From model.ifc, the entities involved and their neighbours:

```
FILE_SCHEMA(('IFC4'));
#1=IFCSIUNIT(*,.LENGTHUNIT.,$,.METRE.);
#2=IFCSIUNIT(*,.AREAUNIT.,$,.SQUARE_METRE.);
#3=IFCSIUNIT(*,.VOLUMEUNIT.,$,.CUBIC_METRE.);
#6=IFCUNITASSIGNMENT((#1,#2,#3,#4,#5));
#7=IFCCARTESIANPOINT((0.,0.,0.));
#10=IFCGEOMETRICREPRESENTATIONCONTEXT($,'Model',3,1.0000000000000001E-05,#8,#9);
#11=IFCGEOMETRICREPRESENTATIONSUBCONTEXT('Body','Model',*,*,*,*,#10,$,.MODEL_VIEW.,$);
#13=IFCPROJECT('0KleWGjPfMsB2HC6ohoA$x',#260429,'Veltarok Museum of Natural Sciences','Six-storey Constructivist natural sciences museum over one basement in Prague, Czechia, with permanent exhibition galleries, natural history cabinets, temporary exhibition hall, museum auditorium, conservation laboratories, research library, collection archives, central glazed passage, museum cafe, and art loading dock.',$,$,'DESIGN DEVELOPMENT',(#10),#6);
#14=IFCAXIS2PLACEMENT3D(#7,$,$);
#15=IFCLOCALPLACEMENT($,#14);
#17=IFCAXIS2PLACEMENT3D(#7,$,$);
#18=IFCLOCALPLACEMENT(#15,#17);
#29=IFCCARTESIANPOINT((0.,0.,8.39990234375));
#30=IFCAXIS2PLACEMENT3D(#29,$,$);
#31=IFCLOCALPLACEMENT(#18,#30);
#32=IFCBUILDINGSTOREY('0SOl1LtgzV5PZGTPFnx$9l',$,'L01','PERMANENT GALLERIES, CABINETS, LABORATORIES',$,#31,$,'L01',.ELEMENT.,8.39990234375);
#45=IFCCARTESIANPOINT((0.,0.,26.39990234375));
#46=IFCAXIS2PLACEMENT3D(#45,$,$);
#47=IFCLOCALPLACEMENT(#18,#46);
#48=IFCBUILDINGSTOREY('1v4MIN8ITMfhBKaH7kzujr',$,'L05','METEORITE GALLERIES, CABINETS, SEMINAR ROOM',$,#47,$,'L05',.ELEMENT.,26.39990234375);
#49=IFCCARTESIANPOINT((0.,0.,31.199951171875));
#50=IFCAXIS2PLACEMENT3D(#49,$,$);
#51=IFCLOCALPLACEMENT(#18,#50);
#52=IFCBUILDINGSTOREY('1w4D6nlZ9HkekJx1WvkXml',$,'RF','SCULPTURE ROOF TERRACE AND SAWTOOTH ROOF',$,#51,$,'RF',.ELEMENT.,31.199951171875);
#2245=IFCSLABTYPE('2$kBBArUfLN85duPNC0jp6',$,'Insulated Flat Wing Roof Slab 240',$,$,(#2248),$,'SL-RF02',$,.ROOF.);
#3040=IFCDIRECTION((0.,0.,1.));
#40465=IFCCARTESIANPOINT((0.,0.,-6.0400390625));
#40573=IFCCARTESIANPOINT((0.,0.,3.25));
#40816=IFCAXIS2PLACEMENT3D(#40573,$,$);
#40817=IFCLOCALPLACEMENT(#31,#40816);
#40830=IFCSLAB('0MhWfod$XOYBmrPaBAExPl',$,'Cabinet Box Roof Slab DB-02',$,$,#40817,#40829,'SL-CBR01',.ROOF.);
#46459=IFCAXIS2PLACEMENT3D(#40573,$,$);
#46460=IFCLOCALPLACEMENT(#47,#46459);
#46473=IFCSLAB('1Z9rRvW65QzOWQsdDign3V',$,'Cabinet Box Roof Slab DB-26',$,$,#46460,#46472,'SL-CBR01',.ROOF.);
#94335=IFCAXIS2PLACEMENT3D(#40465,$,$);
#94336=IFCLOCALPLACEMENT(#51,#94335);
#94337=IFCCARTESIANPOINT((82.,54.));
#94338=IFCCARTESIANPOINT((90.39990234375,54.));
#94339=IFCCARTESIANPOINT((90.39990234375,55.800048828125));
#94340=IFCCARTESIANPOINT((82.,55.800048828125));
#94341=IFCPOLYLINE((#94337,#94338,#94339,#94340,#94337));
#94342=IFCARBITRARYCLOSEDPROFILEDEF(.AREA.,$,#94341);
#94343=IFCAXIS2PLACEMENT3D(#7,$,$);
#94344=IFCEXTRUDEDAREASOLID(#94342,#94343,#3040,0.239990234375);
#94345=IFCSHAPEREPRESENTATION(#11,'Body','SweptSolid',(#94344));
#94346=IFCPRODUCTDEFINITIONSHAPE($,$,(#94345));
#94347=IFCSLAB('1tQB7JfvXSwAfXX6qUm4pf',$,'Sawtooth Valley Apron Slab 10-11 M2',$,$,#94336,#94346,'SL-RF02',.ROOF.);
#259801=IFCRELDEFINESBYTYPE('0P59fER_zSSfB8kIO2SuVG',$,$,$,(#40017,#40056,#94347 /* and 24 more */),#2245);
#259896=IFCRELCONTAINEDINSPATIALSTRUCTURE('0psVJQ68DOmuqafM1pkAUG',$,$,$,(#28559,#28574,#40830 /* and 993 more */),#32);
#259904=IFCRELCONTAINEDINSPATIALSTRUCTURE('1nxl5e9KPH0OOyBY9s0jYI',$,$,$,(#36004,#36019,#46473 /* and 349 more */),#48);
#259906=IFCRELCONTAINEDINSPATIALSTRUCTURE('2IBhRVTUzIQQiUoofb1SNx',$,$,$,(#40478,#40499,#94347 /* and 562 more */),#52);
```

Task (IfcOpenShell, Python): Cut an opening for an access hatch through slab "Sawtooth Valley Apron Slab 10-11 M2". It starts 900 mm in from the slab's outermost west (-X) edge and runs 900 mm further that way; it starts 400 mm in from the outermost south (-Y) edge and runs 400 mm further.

```python
import numpy as np
import ifcopenshell
import ifcopenshell.api.feature
import ifcopenshell.api.geometry
import ifcopenshell.api.root
import ifcopenshell.geom
import ifcopenshell.util.placement
import ifcopenshell.util.representation
import ifcopenshell.util.shape
import ifcopenshell.util.unit

model = ifcopenshell.open("model.ifc")
unit_scale = ifcopenshell.util.unit.calculate_unit_scale(model)
settings = ifcopenshell.geom.settings()


def volume(element):
    """Net volume in cubic metres, openings subtracted."""
    shape = ifcopenshell.geom.create_shape(settings, element)
    return ifcopenshell.util.shape.get_volume(shape.geometry)


slab = model.by_guid("1tQB7JfvXSwAfXX6qUm4pf")
before = volume(slab)

# Extent in the slab's own axes, in metres. The edges named are its -X and -Y sides.
slab_shape = ifcopenshell.geom.create_shape(settings, slab)
vertices = ifcopenshell.util.shape.get_vertices(slab_shape.geometry)
x_min, y_min, bottom = vertices.min(axis=0)
top = vertices[:, 2].max()

opening = ifcopenshell.api.root.create_entity(model, ifc_class="IfcOpeningElement", name="Access hatch opening", predefined_type="OPENING")
context = ifcopenshell.util.representation.get_context(model, "Model", "Body", "MODEL_VIEW")
width, depth = 0.9, 0.4
outline = [(0.0, 0.0), (width, 0.0), (width, depth), (0.0, depth), (0.0, 0.0)]
# Overshoot both faces by 50 mm so the cut is clean.
shape = ifcopenshell.api.geometry.add_slab_representation(
    model, context=context, depth=top - bottom + 0.1, polyline=outline
)
ifcopenshell.api.geometry.assign_representation(model, product=opening, representation=shape)

matrix = ifcopenshell.util.placement.get_local_placement(slab.ObjectPlacement)
matrix[:, 3] = matrix @ np.append(np.array([x_min + 0.9, y_min + 0.4, bottom - 0.05]) / unit_scale, 1.0)
ifcopenshell.api.geometry.edit_object_placement(model, product=opening, matrix=matrix, is_si=False)
ifcopenshell.api.feature.add_feature(model, feature=opening, element=slab)

after = volume(slab)

print(f"slab volume {before:.3f} -> {after:.3f} m3")

model.write("model_edited.ifc")
```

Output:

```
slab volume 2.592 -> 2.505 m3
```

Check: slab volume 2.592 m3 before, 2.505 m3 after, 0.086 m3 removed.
